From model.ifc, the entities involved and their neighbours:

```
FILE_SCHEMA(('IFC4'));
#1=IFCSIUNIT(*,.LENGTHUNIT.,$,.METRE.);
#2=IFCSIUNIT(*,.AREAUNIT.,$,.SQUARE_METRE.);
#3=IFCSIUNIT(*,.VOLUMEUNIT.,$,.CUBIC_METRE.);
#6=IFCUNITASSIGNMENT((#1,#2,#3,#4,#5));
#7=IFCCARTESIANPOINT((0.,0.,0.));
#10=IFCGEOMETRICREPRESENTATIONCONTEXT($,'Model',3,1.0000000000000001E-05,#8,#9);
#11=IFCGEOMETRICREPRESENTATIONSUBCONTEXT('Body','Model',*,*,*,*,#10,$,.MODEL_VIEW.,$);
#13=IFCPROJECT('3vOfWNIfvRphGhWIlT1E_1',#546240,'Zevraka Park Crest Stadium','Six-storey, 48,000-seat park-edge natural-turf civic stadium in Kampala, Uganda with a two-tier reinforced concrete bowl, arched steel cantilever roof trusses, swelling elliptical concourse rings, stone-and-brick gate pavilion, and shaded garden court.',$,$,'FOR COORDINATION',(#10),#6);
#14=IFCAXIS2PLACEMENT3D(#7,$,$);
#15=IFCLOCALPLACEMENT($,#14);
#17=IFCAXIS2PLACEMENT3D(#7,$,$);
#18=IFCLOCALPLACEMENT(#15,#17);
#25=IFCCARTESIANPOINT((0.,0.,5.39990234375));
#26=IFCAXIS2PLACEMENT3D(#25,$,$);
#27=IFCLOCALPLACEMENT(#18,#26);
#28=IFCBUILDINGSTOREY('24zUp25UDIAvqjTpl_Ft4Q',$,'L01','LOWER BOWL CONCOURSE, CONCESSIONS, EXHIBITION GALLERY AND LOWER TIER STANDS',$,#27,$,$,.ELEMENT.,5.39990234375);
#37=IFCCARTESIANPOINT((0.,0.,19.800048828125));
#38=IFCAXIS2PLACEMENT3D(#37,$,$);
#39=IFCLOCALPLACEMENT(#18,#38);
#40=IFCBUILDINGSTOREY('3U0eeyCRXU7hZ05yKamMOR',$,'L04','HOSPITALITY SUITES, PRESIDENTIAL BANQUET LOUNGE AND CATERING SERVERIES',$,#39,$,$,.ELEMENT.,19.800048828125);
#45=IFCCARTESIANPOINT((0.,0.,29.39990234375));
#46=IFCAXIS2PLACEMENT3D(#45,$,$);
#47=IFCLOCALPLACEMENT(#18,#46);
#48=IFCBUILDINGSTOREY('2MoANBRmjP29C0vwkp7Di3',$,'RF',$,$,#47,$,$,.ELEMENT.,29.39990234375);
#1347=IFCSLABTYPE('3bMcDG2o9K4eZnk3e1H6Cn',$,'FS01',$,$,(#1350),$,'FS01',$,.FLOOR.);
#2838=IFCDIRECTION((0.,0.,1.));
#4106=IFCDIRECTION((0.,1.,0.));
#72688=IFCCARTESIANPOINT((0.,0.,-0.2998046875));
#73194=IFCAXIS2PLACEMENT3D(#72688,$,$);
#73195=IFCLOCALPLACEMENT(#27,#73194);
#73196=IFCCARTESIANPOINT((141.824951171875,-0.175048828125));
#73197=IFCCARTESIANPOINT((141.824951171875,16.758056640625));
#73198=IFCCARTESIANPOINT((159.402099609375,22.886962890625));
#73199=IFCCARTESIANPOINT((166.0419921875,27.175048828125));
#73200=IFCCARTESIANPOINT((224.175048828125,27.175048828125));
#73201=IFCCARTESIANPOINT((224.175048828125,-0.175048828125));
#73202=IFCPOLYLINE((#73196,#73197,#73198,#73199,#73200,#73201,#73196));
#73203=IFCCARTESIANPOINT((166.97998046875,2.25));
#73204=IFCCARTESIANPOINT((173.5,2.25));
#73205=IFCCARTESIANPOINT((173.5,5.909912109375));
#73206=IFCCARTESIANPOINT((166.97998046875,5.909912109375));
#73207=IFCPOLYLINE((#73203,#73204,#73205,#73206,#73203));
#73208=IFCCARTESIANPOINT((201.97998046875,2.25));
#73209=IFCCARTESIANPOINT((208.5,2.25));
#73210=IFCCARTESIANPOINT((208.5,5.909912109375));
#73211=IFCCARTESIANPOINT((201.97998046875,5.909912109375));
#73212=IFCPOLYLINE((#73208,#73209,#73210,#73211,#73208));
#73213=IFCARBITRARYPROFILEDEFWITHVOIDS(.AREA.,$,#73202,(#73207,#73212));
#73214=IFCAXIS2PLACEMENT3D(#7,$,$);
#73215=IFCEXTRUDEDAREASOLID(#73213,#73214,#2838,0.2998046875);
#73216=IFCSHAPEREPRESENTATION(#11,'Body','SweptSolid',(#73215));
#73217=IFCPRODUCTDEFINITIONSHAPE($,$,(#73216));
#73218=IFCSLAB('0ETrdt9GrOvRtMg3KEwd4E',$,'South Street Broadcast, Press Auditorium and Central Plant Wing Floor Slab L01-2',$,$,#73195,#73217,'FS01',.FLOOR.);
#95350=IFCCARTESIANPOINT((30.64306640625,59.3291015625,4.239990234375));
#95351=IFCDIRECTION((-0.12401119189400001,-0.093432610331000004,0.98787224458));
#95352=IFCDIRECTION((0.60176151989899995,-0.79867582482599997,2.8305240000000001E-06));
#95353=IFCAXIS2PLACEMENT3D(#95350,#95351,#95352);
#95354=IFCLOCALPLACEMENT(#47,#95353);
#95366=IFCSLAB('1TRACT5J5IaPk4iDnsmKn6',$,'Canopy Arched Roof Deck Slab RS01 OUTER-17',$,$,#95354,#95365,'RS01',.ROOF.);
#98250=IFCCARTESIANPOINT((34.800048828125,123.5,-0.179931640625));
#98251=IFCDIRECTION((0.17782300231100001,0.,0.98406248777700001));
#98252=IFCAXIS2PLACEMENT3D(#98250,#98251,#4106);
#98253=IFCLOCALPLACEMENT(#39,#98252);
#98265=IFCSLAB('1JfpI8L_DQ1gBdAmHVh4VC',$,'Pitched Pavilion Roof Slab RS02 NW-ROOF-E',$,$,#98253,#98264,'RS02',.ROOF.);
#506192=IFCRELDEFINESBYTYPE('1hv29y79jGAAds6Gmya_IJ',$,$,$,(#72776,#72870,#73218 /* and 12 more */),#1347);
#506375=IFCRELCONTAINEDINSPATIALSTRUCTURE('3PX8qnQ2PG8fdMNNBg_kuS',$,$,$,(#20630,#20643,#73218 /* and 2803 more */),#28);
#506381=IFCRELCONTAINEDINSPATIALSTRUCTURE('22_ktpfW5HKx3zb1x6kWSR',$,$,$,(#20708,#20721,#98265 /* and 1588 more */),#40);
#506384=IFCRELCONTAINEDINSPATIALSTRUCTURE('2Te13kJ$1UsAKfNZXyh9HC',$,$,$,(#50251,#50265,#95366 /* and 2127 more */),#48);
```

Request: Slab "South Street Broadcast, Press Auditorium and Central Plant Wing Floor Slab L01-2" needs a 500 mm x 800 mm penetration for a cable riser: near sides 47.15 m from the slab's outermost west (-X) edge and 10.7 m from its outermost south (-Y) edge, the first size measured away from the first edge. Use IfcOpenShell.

```python
import numpy as np
import ifcopenshell
import ifcopenshell.api.feature
import ifcopenshell.api.geometry
import ifcopenshell.api.root
import ifcopenshell.geom
import ifcopenshell.util.placement
import ifcopenshell.util.representation
import ifcopenshell.util.shape
import ifcopenshell.util.unit

model = ifcopenshell.open("model.ifc")
unit_scale = ifcopenshell.util.unit.calculate_unit_scale(model)
settings = ifcopenshell.geom.settings()


def volume(element):
    """Net volume in cubic metres, openings subtracted."""
    shape = ifcopenshell.geom.create_shape(settings, element)
    return ifcopenshell.util.shape.get_volume(shape.geometry)


slab = model.by_guid("0ETrdt9GrOvRtMg3KEwd4E")
before = volume(slab)

# Extent in the slab's own axes, in metres. The edges named are its -X and -Y sides.
slab_shape = ifcopenshell.geom.create_shape(settings, slab)
vertices = ifcopenshell.util.shape.get_vertices(slab_shape.geometry)
x_min, y_min, bottom = vertices.min(axis=0)
top = vertices[:, 2].max()

opening = ifcopenshell.api.root.create_entity(model, ifc_class="IfcOpeningElement", name="Cable riser opening", predefined_type="OPENING")
context = ifcopenshell.util.representation.get_context(model, "Model", "Body", "MODEL_VIEW")
width, depth = 0.5, 0.8
outline = [(0.0, 0.0), (width, 0.0), (width, depth), (0.0, depth), (0.0, 0.0)]
# Overshoot both faces by 50 mm so the cut is clean.
shape = ifcopenshell.api.geometry.add_slab_representation(
    model, context=context, depth=top - bottom + 0.1, polyline=outline
)
ifcopenshell.api.geometry.assign_representation(model, product=opening, representation=shape)

matrix = ifcopenshell.util.placement.get_local_placement(slab.ObjectPlacement)
matrix[:, 3] = matrix @ np.append(np.array([x_min + 47.15, y_min + 10.7, bottom - 0.05]) / unit_scale, 1.0)
ifcopenshell.api.geometry.edit_object_placement(model, product=opening, matrix=matrix, is_si=False)
ifcopenshell.api.feature.add_feature(model, feature=opening, element=slab)

after = volume(slab)

print(f"slab volume {before:.3f} -> {after:.3f} m3")

model.write("model_updated.ifc")
```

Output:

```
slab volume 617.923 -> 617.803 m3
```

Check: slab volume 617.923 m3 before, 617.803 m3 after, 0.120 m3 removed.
